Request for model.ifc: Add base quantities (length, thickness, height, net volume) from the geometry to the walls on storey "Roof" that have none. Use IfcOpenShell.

First a look at what the model holds.

```python
import ifcopenshell
import ifcopenshell.util.element
import ifcopenshell.util.unit

model = ifcopenshell.open("model.ifc")
print(model.schema)
for unit_type in ("LENGTHUNIT", "AREAUNIT", "VOLUMEUNIT"):
    print(unit_type, ifcopenshell.util.unit.calculate_unit_scale(model, unit_type))
storey = next(s for s in model.by_type("IfcBuildingStorey") if s.Name == "Roof")
walls = [e for e in ifcopenshell.util.element.get_decomposition(storey) if e.is_a("IfcWall")]
for e in sorted(walls, key=lambda e: e.id()):
    print(e.id(), e.is_a(), e.Name, list(ifcopenshell.util.element.get_psets(e, qtos_only=True)), sep=" | ")
```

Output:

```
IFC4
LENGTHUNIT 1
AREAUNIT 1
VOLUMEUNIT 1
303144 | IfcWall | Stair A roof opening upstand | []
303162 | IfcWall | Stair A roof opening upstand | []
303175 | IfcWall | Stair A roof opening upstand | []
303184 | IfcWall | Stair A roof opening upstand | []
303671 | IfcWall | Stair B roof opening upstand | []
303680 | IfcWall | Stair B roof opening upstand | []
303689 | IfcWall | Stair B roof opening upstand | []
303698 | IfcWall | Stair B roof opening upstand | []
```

```python
import ifcopenshell
import ifcopenshell.api.pset
import ifcopenshell.geom
import ifcopenshell.util.element
import ifcopenshell.util.shape
import ifcopenshell.util.unit

model = ifcopenshell.open("model.ifc")
unit_scale = ifcopenshell.util.unit.calculate_unit_scale(model)
volume_scale = ifcopenshell.util.unit.calculate_unit_scale(model, "VOLUMEUNIT")
settings = ifcopenshell.geom.settings()

storey = next(s for s in model.by_type("IfcBuildingStorey") if s.Name == "Roof")
walls = [e for e in ifcopenshell.util.element.get_decomposition(storey) if e.is_a("IfcWall")]

for e in sorted(walls, key=lambda e: e.id()):
    if ifcopenshell.util.element.get_psets(e, qtos_only=True, should_inherit=False):
        continue
    # Geometry comes back in metres, in the element's own axes.
    shape = ifcopenshell.geom.create_shape(settings, e)
    values = {
        "Length": ifcopenshell.util.shape.get_x(shape.geometry) / unit_scale,
        "Width": ifcopenshell.util.shape.get_y(shape.geometry) / unit_scale,
        "Height": ifcopenshell.util.shape.get_z(shape.geometry) / unit_scale,
        "NetVolume": ifcopenshell.util.shape.get_volume(shape.geometry) / volume_scale,
    }
    qto = ifcopenshell.api.pset.add_qto(model, product=e, name="Qto_WallBaseQuantities")
    ifcopenshell.api.pset.edit_qto(model, qto=qto, properties=values)
    print(e.id(), {k: round(v, 3) for k, v in values.items()})

model.write("model-out.ifc")
```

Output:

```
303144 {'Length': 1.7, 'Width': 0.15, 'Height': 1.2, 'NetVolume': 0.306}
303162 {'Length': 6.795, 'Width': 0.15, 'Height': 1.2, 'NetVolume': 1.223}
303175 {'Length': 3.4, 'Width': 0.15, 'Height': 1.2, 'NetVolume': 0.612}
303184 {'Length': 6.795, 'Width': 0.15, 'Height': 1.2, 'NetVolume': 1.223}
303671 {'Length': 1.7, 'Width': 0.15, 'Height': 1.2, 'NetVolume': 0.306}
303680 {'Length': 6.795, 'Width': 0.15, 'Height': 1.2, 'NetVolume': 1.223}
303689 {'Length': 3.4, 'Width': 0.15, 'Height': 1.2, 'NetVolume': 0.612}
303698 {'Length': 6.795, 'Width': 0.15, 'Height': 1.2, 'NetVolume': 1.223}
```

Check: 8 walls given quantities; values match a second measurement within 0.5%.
